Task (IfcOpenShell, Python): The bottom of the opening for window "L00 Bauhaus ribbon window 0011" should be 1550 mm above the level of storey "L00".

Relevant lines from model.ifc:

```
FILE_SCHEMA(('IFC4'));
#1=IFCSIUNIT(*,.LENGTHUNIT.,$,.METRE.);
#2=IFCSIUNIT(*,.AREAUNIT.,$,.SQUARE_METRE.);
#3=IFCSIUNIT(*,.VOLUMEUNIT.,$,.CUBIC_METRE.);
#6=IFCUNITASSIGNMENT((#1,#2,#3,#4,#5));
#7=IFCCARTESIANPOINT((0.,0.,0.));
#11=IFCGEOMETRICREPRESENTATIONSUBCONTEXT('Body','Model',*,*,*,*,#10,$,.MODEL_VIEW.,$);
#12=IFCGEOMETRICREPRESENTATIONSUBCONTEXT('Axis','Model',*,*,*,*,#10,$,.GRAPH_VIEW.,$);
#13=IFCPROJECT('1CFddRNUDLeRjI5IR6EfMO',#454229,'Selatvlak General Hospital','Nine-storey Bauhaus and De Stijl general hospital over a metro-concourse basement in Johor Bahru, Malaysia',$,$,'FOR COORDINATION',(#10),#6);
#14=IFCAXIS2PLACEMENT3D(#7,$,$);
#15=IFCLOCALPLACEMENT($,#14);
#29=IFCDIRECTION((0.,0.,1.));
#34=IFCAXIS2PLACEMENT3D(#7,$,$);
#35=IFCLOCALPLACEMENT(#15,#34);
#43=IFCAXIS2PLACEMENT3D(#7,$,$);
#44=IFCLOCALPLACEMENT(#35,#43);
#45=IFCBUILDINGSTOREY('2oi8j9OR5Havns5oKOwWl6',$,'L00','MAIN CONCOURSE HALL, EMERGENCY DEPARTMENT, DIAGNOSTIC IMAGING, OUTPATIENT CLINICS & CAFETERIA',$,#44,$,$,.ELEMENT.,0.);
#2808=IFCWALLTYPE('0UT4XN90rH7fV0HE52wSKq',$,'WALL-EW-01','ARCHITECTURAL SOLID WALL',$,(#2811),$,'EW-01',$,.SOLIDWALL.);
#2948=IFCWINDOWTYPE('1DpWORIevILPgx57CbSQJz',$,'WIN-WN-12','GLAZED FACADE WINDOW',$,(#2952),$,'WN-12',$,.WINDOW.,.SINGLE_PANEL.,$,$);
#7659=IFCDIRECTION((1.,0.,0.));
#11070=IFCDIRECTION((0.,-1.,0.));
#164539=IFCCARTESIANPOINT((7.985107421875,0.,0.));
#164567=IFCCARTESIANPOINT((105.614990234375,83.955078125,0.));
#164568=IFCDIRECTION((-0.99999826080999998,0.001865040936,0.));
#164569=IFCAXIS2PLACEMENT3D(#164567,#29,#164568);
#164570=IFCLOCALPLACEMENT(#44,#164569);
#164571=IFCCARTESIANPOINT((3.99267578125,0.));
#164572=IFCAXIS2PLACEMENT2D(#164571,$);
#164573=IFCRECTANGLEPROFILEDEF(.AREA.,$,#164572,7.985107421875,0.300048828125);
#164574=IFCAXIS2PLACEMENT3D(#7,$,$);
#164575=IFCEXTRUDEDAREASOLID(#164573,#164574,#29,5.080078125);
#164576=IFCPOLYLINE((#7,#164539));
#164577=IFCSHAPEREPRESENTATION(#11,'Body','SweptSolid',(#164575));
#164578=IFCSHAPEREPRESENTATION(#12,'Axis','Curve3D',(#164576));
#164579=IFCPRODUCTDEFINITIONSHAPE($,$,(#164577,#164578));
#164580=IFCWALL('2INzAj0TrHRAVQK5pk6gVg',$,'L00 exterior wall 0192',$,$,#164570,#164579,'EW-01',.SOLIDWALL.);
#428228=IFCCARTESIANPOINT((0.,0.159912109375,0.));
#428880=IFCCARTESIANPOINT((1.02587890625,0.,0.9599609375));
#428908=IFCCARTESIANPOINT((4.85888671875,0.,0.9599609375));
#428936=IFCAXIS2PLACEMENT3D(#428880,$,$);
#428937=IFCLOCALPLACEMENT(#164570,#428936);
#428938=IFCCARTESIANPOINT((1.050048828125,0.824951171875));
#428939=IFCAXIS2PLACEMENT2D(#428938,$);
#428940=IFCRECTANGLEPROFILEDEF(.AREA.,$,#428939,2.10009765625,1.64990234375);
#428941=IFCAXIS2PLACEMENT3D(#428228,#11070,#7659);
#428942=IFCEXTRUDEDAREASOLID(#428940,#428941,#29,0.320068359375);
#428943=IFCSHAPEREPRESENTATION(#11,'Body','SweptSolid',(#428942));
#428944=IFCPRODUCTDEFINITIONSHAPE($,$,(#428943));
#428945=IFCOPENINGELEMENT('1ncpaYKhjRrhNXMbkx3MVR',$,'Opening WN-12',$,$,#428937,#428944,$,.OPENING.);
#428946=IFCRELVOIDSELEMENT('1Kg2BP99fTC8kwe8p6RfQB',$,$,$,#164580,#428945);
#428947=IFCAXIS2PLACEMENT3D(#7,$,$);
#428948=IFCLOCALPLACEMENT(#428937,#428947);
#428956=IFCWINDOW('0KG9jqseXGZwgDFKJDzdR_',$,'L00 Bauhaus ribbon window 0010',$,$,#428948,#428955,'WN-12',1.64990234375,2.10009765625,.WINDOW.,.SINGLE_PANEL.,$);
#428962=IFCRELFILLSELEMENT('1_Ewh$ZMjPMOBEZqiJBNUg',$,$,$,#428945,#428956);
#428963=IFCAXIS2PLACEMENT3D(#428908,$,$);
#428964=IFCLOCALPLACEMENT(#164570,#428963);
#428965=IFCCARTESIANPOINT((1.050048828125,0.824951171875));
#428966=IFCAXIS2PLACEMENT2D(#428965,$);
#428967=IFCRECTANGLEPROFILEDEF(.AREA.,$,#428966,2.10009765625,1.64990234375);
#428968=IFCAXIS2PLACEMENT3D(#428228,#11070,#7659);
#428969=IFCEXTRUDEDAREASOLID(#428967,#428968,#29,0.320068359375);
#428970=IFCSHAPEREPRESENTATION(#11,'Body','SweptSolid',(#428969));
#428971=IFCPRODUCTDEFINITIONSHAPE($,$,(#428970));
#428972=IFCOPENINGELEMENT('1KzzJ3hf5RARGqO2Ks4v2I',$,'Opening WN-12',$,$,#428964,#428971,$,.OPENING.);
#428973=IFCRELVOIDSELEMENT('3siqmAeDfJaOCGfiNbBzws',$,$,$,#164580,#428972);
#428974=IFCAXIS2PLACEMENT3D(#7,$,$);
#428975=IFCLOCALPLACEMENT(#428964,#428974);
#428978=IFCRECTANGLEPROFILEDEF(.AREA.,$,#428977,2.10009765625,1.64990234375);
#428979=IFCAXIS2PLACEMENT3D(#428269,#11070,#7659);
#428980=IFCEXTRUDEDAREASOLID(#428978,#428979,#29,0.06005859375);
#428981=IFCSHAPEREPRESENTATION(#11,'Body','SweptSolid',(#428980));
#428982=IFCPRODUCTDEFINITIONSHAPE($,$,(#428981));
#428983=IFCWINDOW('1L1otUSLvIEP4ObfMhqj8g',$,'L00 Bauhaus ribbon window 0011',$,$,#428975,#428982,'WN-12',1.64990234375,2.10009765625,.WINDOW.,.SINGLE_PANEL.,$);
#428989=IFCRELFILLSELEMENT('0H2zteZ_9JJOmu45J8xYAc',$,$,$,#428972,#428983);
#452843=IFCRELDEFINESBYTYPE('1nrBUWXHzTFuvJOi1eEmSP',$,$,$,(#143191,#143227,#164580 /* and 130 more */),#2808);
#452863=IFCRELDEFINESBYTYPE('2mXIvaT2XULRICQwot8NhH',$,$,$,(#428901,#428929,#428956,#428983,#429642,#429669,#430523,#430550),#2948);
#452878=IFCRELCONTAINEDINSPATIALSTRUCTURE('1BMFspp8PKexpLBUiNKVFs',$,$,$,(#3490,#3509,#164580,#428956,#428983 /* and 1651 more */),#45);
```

```python
import numpy as np
import ifcopenshell
import ifcopenshell.api.geometry
import ifcopenshell.geom
import ifcopenshell.util.element
import ifcopenshell.util.placement
import ifcopenshell.util.shape
import ifcopenshell.util.unit

model = ifcopenshell.open("model.ifc")
unit_scale = ifcopenshell.util.unit.calculate_unit_scale(model)

window = model.by_guid("1L1otUSLvIEP4ObfMhqj8g")
opening = window.FillsVoids[0].RelatingOpeningElement
storey = ifcopenshell.util.element.get_container(window, ifc_class="IfcBuildingStorey")
level = ifcopenshell.util.placement.get_local_placement(storey.ObjectPlacement)[2, 3]

# The opening's origin need not be at the sill, so measure its lowest point.
shape = ifcopenshell.geom.create_shape(ifcopenshell.geom.settings(), opening)
bottom = ifcopenshell.util.shape.get_shape_bottom_elevation(shape, shape.geometry) / unit_scale
dz = level + 1.55 / unit_scale - bottom

shift = np.array([0.0, 0.0, dz])
# The window is placed relative to its opening, so it follows when the opening moves.
matrix = ifcopenshell.util.placement.get_local_placement(opening.ObjectPlacement)
matrix[:3, 3] += shift
ifcopenshell.api.geometry.edit_object_placement(
    model, product=opening, matrix=matrix, is_si=False, should_transform_children=True
)

print(f"moved by {dz * unit_scale:+.3f} m")

model.write("model_rev.ifc")
```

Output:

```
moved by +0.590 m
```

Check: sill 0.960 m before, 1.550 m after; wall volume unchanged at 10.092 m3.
